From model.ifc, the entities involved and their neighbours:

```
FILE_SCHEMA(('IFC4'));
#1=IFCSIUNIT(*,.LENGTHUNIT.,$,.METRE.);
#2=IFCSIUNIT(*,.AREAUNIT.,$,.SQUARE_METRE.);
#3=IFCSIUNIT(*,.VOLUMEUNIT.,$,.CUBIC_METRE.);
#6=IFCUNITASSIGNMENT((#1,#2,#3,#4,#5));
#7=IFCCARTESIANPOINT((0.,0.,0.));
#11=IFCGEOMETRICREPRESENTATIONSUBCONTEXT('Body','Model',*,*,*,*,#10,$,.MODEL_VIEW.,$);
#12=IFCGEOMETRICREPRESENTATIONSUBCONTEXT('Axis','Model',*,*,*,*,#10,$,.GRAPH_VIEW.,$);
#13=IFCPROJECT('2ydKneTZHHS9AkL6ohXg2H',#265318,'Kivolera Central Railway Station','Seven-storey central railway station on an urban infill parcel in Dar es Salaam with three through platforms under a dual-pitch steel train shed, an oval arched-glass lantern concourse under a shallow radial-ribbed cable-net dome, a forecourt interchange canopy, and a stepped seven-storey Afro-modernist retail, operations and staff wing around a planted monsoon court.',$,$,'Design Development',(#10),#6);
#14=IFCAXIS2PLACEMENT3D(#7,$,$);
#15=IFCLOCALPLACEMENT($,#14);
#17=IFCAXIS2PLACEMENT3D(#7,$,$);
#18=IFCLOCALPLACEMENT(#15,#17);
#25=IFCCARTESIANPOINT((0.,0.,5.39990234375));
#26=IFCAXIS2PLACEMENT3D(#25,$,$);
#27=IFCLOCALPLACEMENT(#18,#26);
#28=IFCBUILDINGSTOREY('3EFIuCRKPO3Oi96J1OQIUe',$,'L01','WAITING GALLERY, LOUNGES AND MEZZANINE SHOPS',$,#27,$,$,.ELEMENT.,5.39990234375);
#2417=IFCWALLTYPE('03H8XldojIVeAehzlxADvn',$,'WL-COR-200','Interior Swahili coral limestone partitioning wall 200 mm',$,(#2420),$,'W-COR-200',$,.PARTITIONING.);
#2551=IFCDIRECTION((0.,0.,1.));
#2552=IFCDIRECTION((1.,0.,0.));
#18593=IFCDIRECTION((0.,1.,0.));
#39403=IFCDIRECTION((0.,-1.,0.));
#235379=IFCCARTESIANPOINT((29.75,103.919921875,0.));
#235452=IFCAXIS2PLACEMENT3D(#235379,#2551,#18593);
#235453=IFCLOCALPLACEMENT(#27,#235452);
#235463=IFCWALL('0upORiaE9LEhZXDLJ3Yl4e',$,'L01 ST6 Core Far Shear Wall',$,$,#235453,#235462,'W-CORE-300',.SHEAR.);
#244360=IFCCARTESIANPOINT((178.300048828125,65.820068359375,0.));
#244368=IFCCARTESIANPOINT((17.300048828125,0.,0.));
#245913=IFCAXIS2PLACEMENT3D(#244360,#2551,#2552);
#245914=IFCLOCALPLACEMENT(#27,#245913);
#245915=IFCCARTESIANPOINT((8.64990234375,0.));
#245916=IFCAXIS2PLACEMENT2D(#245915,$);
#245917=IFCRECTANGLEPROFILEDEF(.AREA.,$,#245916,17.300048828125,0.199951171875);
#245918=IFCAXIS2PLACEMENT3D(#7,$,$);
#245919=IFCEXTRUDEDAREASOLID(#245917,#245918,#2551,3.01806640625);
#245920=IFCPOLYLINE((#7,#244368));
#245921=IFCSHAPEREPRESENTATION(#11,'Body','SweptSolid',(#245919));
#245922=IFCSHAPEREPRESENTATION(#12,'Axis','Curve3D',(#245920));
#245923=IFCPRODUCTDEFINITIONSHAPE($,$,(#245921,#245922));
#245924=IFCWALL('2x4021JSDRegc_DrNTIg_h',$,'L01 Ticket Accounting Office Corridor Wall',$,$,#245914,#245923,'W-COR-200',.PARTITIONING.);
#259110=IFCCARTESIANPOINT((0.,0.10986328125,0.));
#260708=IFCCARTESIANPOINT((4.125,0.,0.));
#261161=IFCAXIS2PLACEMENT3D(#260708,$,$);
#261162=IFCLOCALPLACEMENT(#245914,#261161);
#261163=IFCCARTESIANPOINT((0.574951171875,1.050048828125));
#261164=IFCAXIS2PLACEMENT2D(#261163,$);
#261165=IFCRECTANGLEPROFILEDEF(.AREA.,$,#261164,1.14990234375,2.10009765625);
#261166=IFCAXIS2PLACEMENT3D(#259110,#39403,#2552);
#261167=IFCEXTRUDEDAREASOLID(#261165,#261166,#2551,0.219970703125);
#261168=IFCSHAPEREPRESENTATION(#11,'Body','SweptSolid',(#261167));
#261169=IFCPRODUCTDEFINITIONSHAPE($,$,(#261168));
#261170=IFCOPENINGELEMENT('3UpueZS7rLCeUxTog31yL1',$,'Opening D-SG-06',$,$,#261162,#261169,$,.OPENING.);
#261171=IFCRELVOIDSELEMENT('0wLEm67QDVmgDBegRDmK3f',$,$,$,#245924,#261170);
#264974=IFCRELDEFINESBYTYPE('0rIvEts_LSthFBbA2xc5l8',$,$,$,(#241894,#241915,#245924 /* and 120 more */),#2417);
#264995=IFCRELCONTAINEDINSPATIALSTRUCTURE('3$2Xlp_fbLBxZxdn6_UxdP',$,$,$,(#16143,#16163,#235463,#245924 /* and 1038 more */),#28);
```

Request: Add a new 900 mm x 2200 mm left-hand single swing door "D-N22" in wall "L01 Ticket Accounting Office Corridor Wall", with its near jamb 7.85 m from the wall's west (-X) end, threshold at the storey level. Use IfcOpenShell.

```python
import numpy as np
import ifcopenshell
import ifcopenshell.api.feature
import ifcopenshell.api.geometry
import ifcopenshell.api.root
import ifcopenshell.api.spatial
import ifcopenshell.geom
import ifcopenshell.util.element
import ifcopenshell.util.placement
import ifcopenshell.util.representation
import ifcopenshell.util.shape
import ifcopenshell.util.unit

model = ifcopenshell.open("model.ifc")
unit_scale = ifcopenshell.util.unit.calculate_unit_scale(model)
settings = ifcopenshell.geom.settings()


def volume(element):
    """Net volume in cubic metres, openings subtracted."""
    shape = ifcopenshell.geom.create_shape(settings, element)
    return ifcopenshell.util.shape.get_volume(shape.geometry)


wall = model.by_guid("2x4021JSDRegc_DrNTIg_h")
storey = ifcopenshell.util.element.get_container(wall, ifc_class="IfcBuildingStorey")
context = ifcopenshell.util.representation.get_context(model, "Model", "Body", "MODEL_VIEW")
before = volume(wall)

width, height, from_end, sill = 0.9, 2.2, 7.85, 0.0  # metres

# The wall runs along its own X axis, and the end named is its -X end.
wall_shape = ifcopenshell.geom.create_shape(settings, wall)
x, y, z = ifcopenshell.util.shape.get_vertices(wall_shape.geometry).T
start = x.min() + from_end
face, thickness = float(y.min()), float(y.max() - y.min())
wall_matrix = ifcopenshell.util.placement.get_local_placement(wall.ObjectPlacement)
level = ifcopenshell.util.placement.get_local_placement(storey.ObjectPlacement)[2, 3]


def in_wall(x, y):
    """Placement at x, y metres in the wall's axes, at sill height."""
    matrix = wall_matrix.copy()
    matrix[:, 3] = wall_matrix @ np.array([x / unit_scale, y / unit_scale, 0.0, 1.0])
    matrix[2, 3] = level + sill / unit_scale
    return matrix


# Opening: a box that overshoots both wall faces by 50 mm.
opening = ifcopenshell.api.root.create_entity(model, ifc_class="IfcOpeningElement", predefined_type="OPENING")
box = ifcopenshell.api.geometry.add_wall_representation(
    model, context=context, length=width, height=height, thickness=thickness + 0.1
)
ifcopenshell.api.geometry.assign_representation(model, product=opening, representation=box)
ifcopenshell.api.geometry.edit_object_placement(model, product=opening, matrix=in_wall(start, face - 0.05), is_si=False)
ifcopenshell.api.feature.add_feature(model, feature=opening, element=wall)

door = ifcopenshell.api.root.create_entity(model, ifc_class="IfcDoor", name="D-N22", predefined_type="DOOR")
door.OverallWidth, door.OverallHeight = width / unit_scale, height / unit_scale
door.OperationType = "SINGLE_SWING_LEFT"
body = ifcopenshell.api.geometry.add_door_representation(
    model,
    context=context,
    overall_width=door.OverallWidth,
    overall_height=door.OverallHeight,
    operation_type="SINGLE_SWING_LEFT",
    lining_properties={"LiningDepth": thickness / unit_scale, "ThresholdDepth": thickness / unit_scale},
)
ifcopenshell.api.geometry.assign_representation(model, product=door, representation=body)
ifcopenshell.api.spatial.assign_container(model, products=[door], relating_structure=storey)
ifcopenshell.api.feature.add_filling(model, opening=opening, element=door)

# The lining spans the wall, so the door starts at the wall face.
ifcopenshell.api.geometry.edit_object_placement(model, product=door, matrix=in_wall(start, face), is_si=False)

after = volume(wall)

print(f"wall volume {before:.3f} -> {after:.3f} m3")

model.write("model-out.ifc")
```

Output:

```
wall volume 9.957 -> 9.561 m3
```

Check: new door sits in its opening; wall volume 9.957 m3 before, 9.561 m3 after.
